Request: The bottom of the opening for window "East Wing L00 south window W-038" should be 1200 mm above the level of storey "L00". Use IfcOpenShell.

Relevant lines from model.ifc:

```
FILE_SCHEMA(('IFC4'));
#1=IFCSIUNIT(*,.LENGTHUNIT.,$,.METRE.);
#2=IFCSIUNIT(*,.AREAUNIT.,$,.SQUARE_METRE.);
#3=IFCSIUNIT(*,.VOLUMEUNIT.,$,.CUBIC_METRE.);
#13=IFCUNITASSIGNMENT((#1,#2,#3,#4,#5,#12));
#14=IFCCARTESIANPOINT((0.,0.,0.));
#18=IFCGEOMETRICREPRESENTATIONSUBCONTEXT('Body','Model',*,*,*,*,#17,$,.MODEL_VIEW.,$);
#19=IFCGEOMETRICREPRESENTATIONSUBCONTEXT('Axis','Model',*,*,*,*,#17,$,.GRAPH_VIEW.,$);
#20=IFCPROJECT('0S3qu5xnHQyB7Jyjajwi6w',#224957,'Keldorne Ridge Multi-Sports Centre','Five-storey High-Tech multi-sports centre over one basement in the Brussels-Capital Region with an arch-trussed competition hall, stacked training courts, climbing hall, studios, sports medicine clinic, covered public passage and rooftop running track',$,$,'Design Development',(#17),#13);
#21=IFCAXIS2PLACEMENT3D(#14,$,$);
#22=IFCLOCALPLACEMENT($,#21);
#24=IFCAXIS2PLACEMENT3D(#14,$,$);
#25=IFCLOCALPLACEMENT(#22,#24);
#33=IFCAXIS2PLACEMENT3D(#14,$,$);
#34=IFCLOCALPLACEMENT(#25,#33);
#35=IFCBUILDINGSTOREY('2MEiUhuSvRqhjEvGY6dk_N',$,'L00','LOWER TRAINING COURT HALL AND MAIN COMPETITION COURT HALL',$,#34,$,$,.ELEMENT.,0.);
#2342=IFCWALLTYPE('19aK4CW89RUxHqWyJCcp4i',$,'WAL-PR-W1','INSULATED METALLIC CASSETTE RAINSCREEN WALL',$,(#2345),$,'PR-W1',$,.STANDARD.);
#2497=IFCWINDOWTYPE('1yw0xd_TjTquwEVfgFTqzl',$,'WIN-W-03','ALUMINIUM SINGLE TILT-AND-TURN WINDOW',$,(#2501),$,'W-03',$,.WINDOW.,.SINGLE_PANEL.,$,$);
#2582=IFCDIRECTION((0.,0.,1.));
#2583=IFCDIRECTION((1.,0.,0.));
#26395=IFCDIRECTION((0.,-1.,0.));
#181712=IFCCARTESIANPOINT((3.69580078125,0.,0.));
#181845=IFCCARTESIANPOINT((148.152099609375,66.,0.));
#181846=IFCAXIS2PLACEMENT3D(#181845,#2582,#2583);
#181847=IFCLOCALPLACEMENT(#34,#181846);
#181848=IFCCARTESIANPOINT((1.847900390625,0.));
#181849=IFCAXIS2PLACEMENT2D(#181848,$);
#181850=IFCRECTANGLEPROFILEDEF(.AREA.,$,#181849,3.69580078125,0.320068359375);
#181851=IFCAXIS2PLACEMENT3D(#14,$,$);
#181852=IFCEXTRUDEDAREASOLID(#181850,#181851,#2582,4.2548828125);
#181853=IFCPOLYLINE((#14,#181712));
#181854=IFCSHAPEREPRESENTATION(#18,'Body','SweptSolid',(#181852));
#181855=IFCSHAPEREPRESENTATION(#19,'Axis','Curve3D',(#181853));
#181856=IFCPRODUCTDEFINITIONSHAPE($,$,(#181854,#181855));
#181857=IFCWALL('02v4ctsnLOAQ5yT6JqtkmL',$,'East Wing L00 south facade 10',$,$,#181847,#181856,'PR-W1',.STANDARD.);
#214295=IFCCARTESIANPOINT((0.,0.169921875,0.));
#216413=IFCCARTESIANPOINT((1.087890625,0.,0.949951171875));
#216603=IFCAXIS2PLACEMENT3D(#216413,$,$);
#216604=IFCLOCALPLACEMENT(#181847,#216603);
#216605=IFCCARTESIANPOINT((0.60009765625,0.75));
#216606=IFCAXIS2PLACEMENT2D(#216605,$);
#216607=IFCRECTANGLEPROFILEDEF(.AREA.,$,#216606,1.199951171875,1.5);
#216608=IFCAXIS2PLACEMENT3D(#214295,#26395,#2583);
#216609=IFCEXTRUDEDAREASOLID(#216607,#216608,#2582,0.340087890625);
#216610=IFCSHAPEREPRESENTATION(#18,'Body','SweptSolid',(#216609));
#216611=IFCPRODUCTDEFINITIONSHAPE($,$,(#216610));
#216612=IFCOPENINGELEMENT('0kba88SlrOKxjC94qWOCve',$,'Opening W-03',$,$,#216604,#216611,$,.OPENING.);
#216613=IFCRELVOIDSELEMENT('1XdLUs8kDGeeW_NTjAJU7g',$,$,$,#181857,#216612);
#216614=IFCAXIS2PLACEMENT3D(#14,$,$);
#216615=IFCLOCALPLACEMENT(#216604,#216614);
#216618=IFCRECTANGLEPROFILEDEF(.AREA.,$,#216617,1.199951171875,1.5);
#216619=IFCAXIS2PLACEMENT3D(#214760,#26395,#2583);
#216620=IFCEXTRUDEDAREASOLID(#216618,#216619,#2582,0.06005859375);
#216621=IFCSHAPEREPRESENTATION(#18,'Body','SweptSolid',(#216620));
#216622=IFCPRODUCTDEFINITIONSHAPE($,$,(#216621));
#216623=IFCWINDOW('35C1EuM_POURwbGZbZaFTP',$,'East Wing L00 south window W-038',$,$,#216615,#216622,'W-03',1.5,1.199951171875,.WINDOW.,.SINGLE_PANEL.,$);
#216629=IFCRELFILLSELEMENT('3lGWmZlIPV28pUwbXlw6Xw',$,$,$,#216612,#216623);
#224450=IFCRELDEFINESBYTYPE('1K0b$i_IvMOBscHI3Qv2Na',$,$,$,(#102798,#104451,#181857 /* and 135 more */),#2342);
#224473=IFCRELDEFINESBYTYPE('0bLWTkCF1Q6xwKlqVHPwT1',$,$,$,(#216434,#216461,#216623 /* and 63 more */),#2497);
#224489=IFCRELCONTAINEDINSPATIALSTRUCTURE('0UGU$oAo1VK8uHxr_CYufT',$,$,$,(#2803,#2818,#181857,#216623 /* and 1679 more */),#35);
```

```python
import numpy as np
import ifcopenshell
import ifcopenshell.api.geometry
import ifcopenshell.geom
import ifcopenshell.util.element
import ifcopenshell.util.placement
import ifcopenshell.util.shape
import ifcopenshell.util.unit

model = ifcopenshell.open("model.ifc")
unit_scale = ifcopenshell.util.unit.calculate_unit_scale(model)

window = model.by_guid("35C1EuM_POURwbGZbZaFTP")
opening = window.FillsVoids[0].RelatingOpeningElement
storey = ifcopenshell.util.element.get_container(window, ifc_class="IfcBuildingStorey")
level = ifcopenshell.util.placement.get_local_placement(storey.ObjectPlacement)[2, 3]

# The opening's origin need not be at the sill, so measure its lowest point.
shape = ifcopenshell.geom.create_shape(ifcopenshell.geom.settings(), opening)
bottom = ifcopenshell.util.shape.get_shape_bottom_elevation(shape, shape.geometry) / unit_scale
dz = level + 1.2 / unit_scale - bottom

shift = np.array([0.0, 0.0, dz])
# The window is placed relative to its opening, so it follows when the opening moves.
matrix = ifcopenshell.util.placement.get_local_placement(opening.ObjectPlacement)
matrix[:3, 3] += shift
ifcopenshell.api.geometry.edit_object_placement(
    model, product=opening, matrix=matrix, is_si=False, should_transform_children=True
)

print(f"moved by {dz * unit_scale:+.3f} m")

model.write("model_edited.ifc")
```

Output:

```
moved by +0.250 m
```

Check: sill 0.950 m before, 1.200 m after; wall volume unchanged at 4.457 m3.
